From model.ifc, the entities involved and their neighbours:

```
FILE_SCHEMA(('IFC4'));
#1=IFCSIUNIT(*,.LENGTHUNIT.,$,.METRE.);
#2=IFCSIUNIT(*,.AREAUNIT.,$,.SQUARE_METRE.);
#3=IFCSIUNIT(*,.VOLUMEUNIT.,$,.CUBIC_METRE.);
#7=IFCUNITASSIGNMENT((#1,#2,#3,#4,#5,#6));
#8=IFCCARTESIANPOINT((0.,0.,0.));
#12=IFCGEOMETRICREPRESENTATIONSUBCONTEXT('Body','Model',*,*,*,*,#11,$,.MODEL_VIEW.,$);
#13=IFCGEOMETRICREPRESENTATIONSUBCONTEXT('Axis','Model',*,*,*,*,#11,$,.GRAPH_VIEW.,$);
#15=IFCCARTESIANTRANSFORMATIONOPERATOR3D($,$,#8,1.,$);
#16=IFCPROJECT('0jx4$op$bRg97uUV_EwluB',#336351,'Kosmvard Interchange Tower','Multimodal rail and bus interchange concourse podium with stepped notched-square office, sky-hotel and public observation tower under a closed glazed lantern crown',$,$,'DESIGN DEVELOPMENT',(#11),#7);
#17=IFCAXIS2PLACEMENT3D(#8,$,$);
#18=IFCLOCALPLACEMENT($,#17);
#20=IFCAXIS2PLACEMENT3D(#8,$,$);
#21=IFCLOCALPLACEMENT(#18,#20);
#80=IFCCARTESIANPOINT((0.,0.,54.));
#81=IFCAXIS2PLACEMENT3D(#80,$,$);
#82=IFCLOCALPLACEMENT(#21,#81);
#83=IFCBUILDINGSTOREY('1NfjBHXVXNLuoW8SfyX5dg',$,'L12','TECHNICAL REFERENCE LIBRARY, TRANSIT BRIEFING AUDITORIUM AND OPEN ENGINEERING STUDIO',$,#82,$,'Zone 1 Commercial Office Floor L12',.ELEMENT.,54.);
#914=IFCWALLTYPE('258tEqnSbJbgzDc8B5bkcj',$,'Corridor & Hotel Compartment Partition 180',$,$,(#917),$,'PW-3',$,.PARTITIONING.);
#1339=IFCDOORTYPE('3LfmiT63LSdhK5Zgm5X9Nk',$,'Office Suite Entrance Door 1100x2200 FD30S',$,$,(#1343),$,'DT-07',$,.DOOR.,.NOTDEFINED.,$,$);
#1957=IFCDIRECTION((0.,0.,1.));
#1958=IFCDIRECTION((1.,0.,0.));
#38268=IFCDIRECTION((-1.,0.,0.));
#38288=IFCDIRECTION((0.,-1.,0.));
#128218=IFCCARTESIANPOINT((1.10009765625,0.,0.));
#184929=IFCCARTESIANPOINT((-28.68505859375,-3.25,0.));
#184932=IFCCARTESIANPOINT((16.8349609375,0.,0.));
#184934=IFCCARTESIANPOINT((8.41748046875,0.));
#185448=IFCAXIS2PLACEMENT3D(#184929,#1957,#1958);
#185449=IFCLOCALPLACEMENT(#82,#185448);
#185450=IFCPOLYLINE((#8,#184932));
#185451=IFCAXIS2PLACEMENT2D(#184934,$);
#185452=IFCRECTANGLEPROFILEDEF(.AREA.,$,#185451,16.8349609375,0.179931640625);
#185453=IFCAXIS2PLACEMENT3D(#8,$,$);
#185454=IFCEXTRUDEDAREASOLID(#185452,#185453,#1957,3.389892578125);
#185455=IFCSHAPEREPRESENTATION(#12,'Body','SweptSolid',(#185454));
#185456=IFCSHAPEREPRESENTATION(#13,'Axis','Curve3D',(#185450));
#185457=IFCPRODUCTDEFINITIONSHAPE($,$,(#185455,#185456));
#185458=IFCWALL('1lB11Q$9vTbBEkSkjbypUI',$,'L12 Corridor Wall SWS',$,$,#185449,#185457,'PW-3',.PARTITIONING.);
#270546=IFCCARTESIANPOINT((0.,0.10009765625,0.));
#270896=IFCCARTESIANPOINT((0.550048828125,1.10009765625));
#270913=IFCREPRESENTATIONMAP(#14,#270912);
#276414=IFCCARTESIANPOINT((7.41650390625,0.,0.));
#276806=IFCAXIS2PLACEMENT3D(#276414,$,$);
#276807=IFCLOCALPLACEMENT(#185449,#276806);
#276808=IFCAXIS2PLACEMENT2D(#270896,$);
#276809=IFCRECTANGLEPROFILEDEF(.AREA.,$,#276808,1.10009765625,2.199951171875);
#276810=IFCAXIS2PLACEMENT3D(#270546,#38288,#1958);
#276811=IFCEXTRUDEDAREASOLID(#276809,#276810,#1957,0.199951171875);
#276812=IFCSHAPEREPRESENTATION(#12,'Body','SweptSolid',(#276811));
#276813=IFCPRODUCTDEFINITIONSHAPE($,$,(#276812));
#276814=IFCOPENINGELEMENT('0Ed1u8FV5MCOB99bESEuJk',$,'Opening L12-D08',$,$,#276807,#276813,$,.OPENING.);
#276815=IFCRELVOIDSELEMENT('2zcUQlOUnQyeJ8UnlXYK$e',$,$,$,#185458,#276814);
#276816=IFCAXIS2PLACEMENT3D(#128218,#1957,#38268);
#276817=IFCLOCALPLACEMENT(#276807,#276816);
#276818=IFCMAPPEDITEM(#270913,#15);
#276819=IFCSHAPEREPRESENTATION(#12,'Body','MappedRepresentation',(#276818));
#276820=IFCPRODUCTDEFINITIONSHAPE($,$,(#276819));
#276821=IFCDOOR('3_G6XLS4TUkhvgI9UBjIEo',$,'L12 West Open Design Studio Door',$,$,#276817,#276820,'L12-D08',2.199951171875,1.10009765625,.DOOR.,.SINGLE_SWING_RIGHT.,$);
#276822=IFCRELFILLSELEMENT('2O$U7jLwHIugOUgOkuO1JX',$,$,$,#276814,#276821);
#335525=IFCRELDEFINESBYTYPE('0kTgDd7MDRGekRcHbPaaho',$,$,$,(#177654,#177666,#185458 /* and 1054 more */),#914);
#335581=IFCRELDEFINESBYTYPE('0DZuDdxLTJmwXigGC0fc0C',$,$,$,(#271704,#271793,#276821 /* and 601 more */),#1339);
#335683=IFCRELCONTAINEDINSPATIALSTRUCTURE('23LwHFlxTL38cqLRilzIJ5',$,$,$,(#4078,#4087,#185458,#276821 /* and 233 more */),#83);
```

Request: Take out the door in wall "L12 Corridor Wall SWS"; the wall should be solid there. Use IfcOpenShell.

```python
import ifcopenshell
import ifcopenshell.api.feature
import ifcopenshell.api.root
import ifcopenshell.geom
import ifcopenshell.util.shape

model = ifcopenshell.open("model.ifc")
settings = ifcopenshell.geom.settings()


def volume(element):
    """Net volume in cubic metres, openings subtracted."""
    shape = ifcopenshell.geom.create_shape(settings, element)
    return ifcopenshell.util.shape.get_volume(shape.geometry)


door = model.by_guid("3_G6XLS4TUkhvgI9UBjIEo")
opening = door.FillsVoids[0].RelatingOpeningElement
wall = opening.VoidsElements[0].RelatingBuildingElement
before = volume(wall)

ifcopenshell.api.root.remove_product(model, product=door)
ifcopenshell.api.feature.remove_feature(model, feature=opening)

after = volume(wall)

print(f"wall volume {before:.3f} -> {after:.3f} m3")

model.write("model_v2.ifc")
```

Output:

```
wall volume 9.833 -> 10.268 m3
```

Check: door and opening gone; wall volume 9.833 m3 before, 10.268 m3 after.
